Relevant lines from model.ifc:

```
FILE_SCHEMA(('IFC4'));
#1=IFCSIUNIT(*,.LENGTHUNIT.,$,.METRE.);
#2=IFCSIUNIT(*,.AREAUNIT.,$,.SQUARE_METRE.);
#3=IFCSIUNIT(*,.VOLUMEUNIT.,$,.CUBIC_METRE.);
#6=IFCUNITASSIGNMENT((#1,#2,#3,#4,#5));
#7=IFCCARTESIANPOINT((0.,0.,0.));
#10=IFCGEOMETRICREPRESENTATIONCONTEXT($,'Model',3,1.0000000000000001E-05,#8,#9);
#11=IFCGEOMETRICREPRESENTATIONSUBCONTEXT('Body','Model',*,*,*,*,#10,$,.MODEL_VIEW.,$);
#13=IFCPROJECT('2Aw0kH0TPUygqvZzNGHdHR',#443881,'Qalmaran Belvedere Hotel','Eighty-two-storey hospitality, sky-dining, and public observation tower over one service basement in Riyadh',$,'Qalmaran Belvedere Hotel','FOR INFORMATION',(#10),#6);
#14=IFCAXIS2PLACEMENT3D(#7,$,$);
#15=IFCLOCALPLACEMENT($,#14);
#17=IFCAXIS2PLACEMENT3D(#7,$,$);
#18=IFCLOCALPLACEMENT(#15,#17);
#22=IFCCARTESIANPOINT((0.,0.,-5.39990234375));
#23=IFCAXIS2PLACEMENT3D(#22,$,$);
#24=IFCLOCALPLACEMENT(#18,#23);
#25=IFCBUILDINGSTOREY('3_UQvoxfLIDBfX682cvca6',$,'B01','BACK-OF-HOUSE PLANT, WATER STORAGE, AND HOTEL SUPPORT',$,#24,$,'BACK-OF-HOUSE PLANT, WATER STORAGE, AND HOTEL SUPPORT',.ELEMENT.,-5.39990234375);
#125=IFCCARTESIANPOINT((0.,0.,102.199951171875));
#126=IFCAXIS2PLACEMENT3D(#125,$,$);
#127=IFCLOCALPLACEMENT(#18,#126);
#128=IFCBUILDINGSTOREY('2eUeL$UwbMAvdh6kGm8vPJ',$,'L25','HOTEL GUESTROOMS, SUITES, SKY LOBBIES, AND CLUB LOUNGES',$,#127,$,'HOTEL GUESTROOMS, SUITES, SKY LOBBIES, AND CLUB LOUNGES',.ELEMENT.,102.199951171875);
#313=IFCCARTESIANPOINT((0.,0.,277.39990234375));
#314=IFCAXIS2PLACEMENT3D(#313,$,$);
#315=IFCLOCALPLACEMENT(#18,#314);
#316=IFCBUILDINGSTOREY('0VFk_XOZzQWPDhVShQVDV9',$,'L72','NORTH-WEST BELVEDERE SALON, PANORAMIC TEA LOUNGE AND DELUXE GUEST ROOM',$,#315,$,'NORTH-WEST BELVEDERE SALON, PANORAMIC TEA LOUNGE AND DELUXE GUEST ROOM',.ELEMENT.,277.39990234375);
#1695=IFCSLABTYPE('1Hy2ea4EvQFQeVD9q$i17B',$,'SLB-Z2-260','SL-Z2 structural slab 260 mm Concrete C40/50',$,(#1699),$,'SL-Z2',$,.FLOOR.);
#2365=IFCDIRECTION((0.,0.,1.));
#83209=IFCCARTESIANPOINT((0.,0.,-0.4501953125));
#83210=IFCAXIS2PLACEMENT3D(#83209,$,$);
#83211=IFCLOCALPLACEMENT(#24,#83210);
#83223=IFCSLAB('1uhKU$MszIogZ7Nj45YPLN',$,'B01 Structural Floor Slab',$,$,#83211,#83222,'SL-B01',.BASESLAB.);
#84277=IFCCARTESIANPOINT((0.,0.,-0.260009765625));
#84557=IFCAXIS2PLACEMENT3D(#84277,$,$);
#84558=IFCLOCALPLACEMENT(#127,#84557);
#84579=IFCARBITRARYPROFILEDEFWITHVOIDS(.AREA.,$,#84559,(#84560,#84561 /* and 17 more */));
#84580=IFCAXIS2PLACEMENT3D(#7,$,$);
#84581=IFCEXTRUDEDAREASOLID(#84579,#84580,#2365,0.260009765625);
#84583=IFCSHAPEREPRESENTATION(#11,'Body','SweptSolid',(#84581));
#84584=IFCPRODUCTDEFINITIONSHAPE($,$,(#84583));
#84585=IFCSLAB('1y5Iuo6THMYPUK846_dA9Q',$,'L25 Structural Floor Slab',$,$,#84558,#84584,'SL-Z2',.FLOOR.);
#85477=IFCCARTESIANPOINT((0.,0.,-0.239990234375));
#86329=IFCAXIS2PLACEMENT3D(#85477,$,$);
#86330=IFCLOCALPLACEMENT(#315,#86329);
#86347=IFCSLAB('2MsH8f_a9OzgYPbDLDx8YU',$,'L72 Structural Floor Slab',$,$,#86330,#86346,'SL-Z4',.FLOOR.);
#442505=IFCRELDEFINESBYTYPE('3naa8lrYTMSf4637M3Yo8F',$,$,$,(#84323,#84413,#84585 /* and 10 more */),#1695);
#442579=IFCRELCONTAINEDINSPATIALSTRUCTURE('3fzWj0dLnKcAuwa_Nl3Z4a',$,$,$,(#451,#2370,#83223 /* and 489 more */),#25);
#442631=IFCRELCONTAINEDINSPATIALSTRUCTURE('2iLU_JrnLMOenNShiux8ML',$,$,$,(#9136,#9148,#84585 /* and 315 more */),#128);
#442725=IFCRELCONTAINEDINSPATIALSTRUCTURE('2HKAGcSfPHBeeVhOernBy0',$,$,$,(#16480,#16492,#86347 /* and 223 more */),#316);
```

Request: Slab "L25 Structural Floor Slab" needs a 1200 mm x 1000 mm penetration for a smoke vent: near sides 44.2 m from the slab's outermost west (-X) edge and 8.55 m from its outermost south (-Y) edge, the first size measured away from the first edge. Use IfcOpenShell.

```python
import numpy as np
import ifcopenshell
import ifcopenshell.api.feature
import ifcopenshell.api.geometry
import ifcopenshell.api.root
import ifcopenshell.geom
import ifcopenshell.util.placement
import ifcopenshell.util.representation
import ifcopenshell.util.shape
import ifcopenshell.util.unit

model = ifcopenshell.open("model.ifc")
unit_scale = ifcopenshell.util.unit.calculate_unit_scale(model)
settings = ifcopenshell.geom.settings()


def volume(element):
    """Net volume in cubic metres, openings subtracted."""
    shape = ifcopenshell.geom.create_shape(settings, element)
    return ifcopenshell.util.shape.get_volume(shape.geometry)


slab = model.by_id(84585)
before = volume(slab)

# Extent in the slab's own axes, in metres. The edges named are its -X and -Y sides.
slab_shape = ifcopenshell.geom.create_shape(settings, slab)
vertices = ifcopenshell.util.shape.get_vertices(slab_shape.geometry)
x_min, y_min, bottom = vertices.min(axis=0)
top = vertices[:, 2].max()

opening = ifcopenshell.api.root.create_entity(model, ifc_class="IfcOpeningElement", name="Smoke vent opening", predefined_type="OPENING")
context = ifcopenshell.util.representation.get_context(model, "Model", "Body", "MODEL_VIEW")
width, depth = 1.2, 1
outline = [(0.0, 0.0), (width, 0.0), (width, depth), (0.0, depth), (0.0, 0.0)]
# Overshoot both faces by 50 mm so the cut is clean.
shape = ifcopenshell.api.geometry.add_slab_representation(
    model, context=context, depth=top - bottom + 0.1, polyline=outline
)
ifcopenshell.api.geometry.assign_representation(model, product=opening, representation=shape)

matrix = ifcopenshell.util.placement.get_local_placement(slab.ObjectPlacement)
matrix[:, 3] = matrix @ np.append(np.array([x_min + 44.2, y_min + 8.55, bottom - 0.05]) / unit_scale, 1.0)
ifcopenshell.api.geometry.edit_object_placement(model, product=opening, matrix=matrix, is_si=False)
ifcopenshell.api.feature.add_feature(model, feature=opening, element=slab)

after = volume(slab)

print(f"slab volume {before:.3f} -> {after:.3f} m3")

model.write("model_rev.ifc")
```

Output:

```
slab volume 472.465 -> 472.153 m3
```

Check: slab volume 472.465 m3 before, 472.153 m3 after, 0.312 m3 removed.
